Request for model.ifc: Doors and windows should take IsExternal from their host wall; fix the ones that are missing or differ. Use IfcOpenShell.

First a look at what the model holds.

```python
import ifcopenshell
import ifcopenshell.util.element

model = ifcopenshell.open("model.ifc")
print(model.schema)
seen = {}
for e in model.by_type("IfcDoor") + model.by_type("IfcWindow"):
    if not e.FillsVoids:
        continue
    host = e.FillsVoids[0].RelatingOpeningElement.VoidsElements[0].RelatingBuildingElement
    own = ifcopenshell.util.element.get_pset(e, f"Pset_{e.is_a()[3:].removesuffix('StandardCase')}Common", "IsExternal")
    wall = ifcopenshell.util.element.get_pset(host, "Pset_WallCommon", "IsExternal")
    seen[e.is_a(), own, wall] = seen.get((e.is_a(), own, wall), 0) + 1
for (cls, own, wall), count in sorted(seen.items(), key=str):
    print(count, cls, "IsExternal:", own, "| host wall:", wall)
```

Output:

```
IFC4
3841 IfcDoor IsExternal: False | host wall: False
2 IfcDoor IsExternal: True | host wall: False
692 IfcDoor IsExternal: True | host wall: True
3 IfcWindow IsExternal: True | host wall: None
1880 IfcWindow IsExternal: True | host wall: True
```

```python
import ifcopenshell
import ifcopenshell.api.pset
import ifcopenshell.util.element

model = ifcopenshell.open("model.ifc")

count = 0
for ifc_class, pset_name in (("IfcDoor", "Pset_DoorCommon"), ("IfcWindow", "Pset_WindowCommon")):
    for e in model.by_type(ifc_class):
        if not e.FillsVoids:
            continue
        host = e.FillsVoids[0].RelatingOpeningElement.VoidsElements[0].RelatingBuildingElement
        external = ifcopenshell.util.element.get_pset(host, "Pset_WallCommon", "IsExternal")
        if external is None or ifcopenshell.util.element.get_pset(e, pset_name, "IsExternal") == external:
            continue
        found = ifcopenshell.util.element.get_pset(e, pset_name, should_inherit=False)
        if found:
            pset = model.by_id(found["id"])
            if len(ifcopenshell.util.element.get_elements_by_pset(pset)) > 1:
                pset = ifcopenshell.api.pset.unshare_pset(model, products=[e], pset=pset)[0]
        else:
            pset = ifcopenshell.api.pset.add_pset(model, product=e, name=pset_name)
        ifcopenshell.api.pset.edit_pset(model, pset=pset, properties={"IsExternal": external})
        count += 1

print(count, "updated")

model.write("model_edited.ifc")
```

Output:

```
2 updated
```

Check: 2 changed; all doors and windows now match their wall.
